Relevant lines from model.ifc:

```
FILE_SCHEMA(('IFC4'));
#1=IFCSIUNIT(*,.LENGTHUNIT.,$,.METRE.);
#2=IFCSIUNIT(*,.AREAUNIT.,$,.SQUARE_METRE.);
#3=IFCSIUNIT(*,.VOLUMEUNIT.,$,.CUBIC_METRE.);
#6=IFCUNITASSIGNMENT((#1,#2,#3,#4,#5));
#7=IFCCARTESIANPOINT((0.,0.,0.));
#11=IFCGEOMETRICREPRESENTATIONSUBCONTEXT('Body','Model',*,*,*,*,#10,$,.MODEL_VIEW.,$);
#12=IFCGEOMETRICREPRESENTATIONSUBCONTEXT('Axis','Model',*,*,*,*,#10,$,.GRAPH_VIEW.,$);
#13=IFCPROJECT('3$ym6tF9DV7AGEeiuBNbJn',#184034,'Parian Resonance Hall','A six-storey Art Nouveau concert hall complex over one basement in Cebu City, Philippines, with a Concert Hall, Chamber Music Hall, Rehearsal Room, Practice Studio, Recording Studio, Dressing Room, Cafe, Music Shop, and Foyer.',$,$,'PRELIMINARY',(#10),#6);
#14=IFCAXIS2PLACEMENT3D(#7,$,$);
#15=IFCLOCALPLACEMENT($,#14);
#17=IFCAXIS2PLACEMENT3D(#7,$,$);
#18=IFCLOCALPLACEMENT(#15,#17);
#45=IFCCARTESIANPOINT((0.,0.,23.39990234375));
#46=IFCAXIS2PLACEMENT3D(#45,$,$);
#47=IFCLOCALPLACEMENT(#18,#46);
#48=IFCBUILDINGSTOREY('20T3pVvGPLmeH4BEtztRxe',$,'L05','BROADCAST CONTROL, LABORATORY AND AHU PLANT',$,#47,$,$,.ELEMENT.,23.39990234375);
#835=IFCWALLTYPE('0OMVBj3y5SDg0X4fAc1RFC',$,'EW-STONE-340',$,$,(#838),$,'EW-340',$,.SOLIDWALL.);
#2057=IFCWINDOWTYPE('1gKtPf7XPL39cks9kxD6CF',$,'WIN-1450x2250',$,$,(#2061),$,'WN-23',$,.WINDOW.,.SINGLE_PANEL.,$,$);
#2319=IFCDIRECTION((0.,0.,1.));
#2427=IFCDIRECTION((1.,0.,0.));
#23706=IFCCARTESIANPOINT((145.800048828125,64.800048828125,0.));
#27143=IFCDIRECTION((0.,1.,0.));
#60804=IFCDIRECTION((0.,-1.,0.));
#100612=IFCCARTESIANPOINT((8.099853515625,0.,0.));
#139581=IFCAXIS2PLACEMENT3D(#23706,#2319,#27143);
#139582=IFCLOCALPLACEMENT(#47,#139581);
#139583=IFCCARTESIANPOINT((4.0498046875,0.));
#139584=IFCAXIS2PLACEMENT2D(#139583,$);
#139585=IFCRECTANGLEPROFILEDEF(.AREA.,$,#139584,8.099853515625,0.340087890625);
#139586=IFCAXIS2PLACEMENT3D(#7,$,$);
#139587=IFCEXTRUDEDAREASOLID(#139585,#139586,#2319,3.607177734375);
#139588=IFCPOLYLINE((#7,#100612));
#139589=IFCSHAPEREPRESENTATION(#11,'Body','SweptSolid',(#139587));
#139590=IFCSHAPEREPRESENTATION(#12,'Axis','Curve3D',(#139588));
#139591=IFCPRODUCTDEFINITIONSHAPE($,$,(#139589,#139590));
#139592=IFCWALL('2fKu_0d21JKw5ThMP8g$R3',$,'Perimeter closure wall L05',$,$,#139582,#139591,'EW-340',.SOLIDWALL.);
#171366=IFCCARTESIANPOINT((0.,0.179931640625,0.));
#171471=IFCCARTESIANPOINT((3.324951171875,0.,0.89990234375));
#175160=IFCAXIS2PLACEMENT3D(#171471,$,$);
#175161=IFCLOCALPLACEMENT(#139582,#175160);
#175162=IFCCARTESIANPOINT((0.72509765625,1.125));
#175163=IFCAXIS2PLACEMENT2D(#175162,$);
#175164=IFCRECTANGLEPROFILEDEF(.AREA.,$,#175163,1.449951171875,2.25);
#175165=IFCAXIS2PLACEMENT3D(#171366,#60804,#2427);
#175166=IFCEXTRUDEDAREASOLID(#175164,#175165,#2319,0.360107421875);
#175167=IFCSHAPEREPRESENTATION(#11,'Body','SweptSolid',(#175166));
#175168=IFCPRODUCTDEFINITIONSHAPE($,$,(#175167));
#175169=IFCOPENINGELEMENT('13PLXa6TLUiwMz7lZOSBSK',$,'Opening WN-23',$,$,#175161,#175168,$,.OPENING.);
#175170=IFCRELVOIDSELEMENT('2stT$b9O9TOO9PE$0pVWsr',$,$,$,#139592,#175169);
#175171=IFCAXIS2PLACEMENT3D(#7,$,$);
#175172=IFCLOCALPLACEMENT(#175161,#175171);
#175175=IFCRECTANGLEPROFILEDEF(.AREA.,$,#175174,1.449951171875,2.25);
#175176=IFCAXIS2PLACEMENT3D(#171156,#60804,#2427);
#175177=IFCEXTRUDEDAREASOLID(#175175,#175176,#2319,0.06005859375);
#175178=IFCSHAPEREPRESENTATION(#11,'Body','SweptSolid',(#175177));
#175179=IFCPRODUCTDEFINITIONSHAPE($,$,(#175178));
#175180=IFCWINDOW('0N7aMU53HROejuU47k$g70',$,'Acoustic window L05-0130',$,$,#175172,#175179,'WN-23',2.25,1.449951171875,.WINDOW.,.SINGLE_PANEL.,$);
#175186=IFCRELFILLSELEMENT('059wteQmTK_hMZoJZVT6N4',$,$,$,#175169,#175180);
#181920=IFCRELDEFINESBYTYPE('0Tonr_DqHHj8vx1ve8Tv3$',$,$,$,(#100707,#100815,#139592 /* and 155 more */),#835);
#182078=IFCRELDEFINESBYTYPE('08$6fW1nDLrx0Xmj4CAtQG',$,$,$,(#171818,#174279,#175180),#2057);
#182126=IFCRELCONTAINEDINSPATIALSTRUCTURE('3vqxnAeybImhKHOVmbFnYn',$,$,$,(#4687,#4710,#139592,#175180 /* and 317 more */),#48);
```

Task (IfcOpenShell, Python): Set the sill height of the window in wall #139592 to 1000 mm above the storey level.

```python
import numpy as np
import ifcopenshell
import ifcopenshell.api.geometry
import ifcopenshell.geom
import ifcopenshell.util.element
import ifcopenshell.util.placement
import ifcopenshell.util.shape
import ifcopenshell.util.unit

model = ifcopenshell.open("model.ifc")
unit_scale = ifcopenshell.util.unit.calculate_unit_scale(model)

window = model.by_id(175180)
opening = window.FillsVoids[0].RelatingOpeningElement
storey = ifcopenshell.util.element.get_container(window, ifc_class="IfcBuildingStorey")
level = ifcopenshell.util.placement.get_local_placement(storey.ObjectPlacement)[2, 3]

# The opening's origin need not be at the sill, so measure its lowest point.
shape = ifcopenshell.geom.create_shape(ifcopenshell.geom.settings(), opening)
bottom = ifcopenshell.util.shape.get_shape_bottom_elevation(shape, shape.geometry) / unit_scale
dz = level + 1 / unit_scale - bottom

shift = np.array([0.0, 0.0, dz])
# The window is placed relative to its opening, so it follows when the opening moves.
matrix = ifcopenshell.util.placement.get_local_placement(opening.ObjectPlacement)
matrix[:3, 3] += shift
ifcopenshell.api.geometry.edit_object_placement(
    model, product=opening, matrix=matrix, is_si=False, should_transform_children=True
)

print(f"moved by {dz * unit_scale:+.3f} m")

model.write("model_updated.ifc")
```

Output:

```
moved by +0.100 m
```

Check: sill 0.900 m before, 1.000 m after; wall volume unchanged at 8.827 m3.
